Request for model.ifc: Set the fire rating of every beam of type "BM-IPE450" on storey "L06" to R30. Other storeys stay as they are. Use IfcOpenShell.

First a look at what the model holds.

```python
import ifcopenshell
import ifcopenshell.util.element

model = ifcopenshell.open("model.ifc")
print(model.schema)
storey = next(s for s in model.by_type("IfcBuildingStorey") if s.Name == "L06")
beams = [e for e in ifcopenshell.util.element.get_decomposition(storey) if e.is_a("IfcBeam")]
seen = {}
for e in beams:
    element_type = ifcopenshell.util.element.get_type(e)
    key = (element_type.Name if element_type != e and element_type else None, ifcopenshell.util.element.get_pset(e, "Pset_BeamCommon", "FireRating"))
    seen[key] = seen.get(key, 0) + 1
for (name, value), count in sorted(seen.items(), key=str):
    print(count, "x", name, "|", value)
```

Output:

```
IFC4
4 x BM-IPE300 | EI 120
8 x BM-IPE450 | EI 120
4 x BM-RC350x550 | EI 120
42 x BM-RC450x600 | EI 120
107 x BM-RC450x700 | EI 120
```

```python
import ifcopenshell
import ifcopenshell.api.pset
import ifcopenshell.util.element

model = ifcopenshell.open("model.ifc")

storey = next(s for s in model.by_type("IfcBuildingStorey") if s.Name == "L06")
beams = [e for e in ifcopenshell.util.element.get_decomposition(storey) if e.is_a("IfcBeam")]

count = 0
for e in beams:
    element_type = ifcopenshell.util.element.get_type(e)
    if element_type in (None, e) or element_type.Name != "BM-IPE450":
        continue
    # add_pset returns the element's existing set when there is one.
    pset = ifcopenshell.api.pset.add_pset(model, product=e, name="Pset_BeamCommon")
    ifcopenshell.api.pset.edit_pset(model, pset=pset, properties={"FireRating": "R30"})
    count += 1

print(count, "beams updated")

model.write("model_rev.ifc")
```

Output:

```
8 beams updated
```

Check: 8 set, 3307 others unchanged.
